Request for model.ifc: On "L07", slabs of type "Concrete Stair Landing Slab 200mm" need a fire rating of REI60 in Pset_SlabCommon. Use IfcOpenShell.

First a look at what the model holds.

```python
import ifcopenshell
import ifcopenshell.util.element

model = ifcopenshell.open("model.ifc")
print(model.schema)
storey = next(s for s in model.by_type("IfcBuildingStorey") if s.Name == "L07")
slabs = [e for e in ifcopenshell.util.element.get_decomposition(storey) if e.is_a("IfcSlab")]
seen = {}
for e in slabs:
    element_type = ifcopenshell.util.element.get_type(e)
    key = (element_type.Name if element_type != e and element_type else None, ifcopenshell.util.element.get_pset(e, "Pset_SlabCommon", "FireRating"))
    seen[key] = seen.get(key, 0) + 1
for (name, value), count in sorted(seen.items(), key=str):
    print(count, "x", name, "|", value)
```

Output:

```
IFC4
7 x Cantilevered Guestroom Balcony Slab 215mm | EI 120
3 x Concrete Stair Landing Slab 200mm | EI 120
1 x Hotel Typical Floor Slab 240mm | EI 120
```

```python
import ifcopenshell
import ifcopenshell.api.pset
import ifcopenshell.util.element

model = ifcopenshell.open("model.ifc")

storey = next(s for s in model.by_type("IfcBuildingStorey") if s.Name == "L07")
slabs = [e for e in ifcopenshell.util.element.get_decomposition(storey) if e.is_a("IfcSlab")]

count = 0
for e in slabs:
    element_type = ifcopenshell.util.element.get_type(e)
    if element_type in (None, e) or element_type.Name != "Concrete Stair Landing Slab 200mm":
        continue
    # add_pset returns the element's existing set when there is one.
    pset = ifcopenshell.api.pset.add_pset(model, product=e, name="Pset_SlabCommon")
    ifcopenshell.api.pset.edit_pset(model, pset=pset, properties={"FireRating": "REI60"})
    count += 1

print(count, "slabs updated")

model.write("model_edited.ifc")
```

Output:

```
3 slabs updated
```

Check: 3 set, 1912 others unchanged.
